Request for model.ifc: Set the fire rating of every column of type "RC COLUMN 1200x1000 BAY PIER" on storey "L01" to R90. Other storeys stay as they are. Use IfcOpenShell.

First a look at what the model holds.

```python
import ifcopenshell
import ifcopenshell.util.element

model = ifcopenshell.open("model.ifc")
print(model.schema)
storey = next(s for s in model.by_type("IfcBuildingStorey") if s.Name == "L01")
columns = [e for e in ifcopenshell.util.element.get_decomposition(storey) if e.is_a("IfcColumn")]
seen = {}
for e in columns:
    element_type = ifcopenshell.util.element.get_type(e)
    key = (element_type.Name if element_type != e and element_type else None, ifcopenshell.util.element.get_pset(e, "Pset_ColumnCommon", "FireRating"))
    seen[key] = seen.get(key, 0) + 1
for (name, value), count in sorted(seen.items(), key=str):
    print(count, "x", name, "|", value)
```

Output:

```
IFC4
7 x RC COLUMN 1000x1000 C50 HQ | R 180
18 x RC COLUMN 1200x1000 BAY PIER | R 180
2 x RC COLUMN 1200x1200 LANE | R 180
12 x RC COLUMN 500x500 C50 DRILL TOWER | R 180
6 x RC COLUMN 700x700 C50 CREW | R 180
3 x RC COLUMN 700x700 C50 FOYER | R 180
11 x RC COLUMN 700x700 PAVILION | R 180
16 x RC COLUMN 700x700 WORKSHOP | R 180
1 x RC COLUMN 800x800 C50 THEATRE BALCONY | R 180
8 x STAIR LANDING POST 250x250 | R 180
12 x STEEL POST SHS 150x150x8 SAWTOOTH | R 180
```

```python
import ifcopenshell
import ifcopenshell.api.pset
import ifcopenshell.util.element

model = ifcopenshell.open("model.ifc")

storey = next(s for s in model.by_type("IfcBuildingStorey") if s.Name == "L01")
columns = [e for e in ifcopenshell.util.element.get_decomposition(storey) if e.is_a("IfcColumn")]

count = 0
for e in columns:
    element_type = ifcopenshell.util.element.get_type(e)
    if element_type in (None, e) or element_type.Name != "RC COLUMN 1200x1000 BAY PIER":
        continue
    # add_pset returns the element's existing set when there is one.
    pset = ifcopenshell.api.pset.add_pset(model, product=e, name="Pset_ColumnCommon")
    ifcopenshell.api.pset.edit_pset(model, pset=pset, properties={"FireRating": "R90"})
    count += 1

print(count, "columns updated")

model.write("model_updated.ifc")
```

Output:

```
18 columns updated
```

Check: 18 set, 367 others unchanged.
